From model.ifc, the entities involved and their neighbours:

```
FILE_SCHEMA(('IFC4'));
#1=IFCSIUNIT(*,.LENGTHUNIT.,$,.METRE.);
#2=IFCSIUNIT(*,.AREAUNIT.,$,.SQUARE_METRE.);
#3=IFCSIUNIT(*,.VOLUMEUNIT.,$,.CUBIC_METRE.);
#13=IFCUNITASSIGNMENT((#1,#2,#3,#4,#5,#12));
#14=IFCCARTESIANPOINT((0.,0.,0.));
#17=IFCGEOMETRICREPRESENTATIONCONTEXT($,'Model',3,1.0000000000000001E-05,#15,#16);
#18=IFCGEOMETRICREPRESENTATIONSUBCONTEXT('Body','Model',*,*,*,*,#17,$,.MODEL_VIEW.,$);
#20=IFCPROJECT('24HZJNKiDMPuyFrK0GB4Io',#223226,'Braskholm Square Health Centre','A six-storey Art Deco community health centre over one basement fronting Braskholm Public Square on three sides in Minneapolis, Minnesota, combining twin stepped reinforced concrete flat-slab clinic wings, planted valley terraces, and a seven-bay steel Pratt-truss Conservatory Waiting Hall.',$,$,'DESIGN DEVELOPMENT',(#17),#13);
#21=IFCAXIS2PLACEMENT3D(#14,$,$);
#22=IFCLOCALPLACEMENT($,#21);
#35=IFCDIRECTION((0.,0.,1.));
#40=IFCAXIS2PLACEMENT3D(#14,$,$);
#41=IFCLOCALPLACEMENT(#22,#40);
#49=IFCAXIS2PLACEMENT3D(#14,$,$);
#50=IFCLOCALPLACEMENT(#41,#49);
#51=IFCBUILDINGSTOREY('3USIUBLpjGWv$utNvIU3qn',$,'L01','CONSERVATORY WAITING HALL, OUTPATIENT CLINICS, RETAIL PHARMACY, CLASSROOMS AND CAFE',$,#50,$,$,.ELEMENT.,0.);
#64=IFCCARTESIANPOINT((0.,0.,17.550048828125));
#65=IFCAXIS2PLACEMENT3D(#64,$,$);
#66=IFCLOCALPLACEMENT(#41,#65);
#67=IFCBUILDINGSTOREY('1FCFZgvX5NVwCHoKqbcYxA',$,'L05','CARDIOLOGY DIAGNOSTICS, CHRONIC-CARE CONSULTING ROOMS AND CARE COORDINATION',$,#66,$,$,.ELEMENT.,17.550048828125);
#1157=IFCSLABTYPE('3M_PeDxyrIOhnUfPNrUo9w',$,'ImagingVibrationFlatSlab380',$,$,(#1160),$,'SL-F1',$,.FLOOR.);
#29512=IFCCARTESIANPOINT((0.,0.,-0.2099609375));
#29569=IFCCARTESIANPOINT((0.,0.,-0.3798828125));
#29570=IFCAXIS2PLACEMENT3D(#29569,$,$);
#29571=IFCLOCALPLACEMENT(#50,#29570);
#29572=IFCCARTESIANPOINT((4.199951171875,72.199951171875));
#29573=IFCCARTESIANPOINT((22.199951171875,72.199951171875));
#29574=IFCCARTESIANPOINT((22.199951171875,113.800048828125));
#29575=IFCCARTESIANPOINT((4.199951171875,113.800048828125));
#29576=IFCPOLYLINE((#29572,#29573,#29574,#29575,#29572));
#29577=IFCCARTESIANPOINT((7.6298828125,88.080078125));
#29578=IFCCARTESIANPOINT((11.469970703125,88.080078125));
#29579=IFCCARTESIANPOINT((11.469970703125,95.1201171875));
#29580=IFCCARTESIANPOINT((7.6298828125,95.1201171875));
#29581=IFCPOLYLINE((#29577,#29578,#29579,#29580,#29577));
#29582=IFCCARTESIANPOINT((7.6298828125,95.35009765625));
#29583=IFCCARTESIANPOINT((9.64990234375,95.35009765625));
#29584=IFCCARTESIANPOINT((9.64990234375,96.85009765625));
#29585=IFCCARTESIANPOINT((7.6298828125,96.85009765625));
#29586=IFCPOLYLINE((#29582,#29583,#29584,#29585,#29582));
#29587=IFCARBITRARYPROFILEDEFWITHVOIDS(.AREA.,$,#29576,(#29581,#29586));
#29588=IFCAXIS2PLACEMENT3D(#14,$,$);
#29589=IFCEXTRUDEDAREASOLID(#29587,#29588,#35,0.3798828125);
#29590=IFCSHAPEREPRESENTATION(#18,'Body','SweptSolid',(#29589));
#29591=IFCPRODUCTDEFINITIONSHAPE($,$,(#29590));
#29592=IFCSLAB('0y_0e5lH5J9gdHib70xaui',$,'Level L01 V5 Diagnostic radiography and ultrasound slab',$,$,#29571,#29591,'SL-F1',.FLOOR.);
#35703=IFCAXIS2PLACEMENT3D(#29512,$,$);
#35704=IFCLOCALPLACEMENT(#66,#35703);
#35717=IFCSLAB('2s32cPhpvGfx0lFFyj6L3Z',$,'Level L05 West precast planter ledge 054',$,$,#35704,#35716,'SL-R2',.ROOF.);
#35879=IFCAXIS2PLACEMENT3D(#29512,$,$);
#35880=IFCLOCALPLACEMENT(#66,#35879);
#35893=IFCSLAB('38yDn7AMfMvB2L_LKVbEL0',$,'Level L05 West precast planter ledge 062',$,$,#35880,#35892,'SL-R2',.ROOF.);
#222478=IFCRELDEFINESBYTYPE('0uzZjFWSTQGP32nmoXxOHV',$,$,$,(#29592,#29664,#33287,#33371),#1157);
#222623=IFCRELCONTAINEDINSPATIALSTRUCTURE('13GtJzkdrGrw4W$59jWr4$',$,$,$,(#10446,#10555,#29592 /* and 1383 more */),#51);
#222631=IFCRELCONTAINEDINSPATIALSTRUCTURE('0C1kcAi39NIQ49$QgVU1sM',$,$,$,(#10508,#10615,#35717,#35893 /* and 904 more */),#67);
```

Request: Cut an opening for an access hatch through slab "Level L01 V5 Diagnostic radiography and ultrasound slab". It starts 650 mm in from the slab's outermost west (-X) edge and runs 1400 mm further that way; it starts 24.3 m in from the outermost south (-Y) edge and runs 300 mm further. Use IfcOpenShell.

```python
import numpy as np
import ifcopenshell
import ifcopenshell.api.feature
import ifcopenshell.api.geometry
import ifcopenshell.api.root
import ifcopenshell.geom
import ifcopenshell.util.placement
import ifcopenshell.util.representation
import ifcopenshell.util.shape
import ifcopenshell.util.unit

model = ifcopenshell.open("model.ifc")
unit_scale = ifcopenshell.util.unit.calculate_unit_scale(model)
settings = ifcopenshell.geom.settings()


def volume(element):
    """Net volume in cubic metres, openings subtracted."""
    shape = ifcopenshell.geom.create_shape(settings, element)
    return ifcopenshell.util.shape.get_volume(shape.geometry)


slab = model.by_guid("0y_0e5lH5J9gdHib70xaui")
before = volume(slab)

# Extent in the slab's own axes, in metres. The edges named are its -X and -Y sides.
slab_shape = ifcopenshell.geom.create_shape(settings, slab)
vertices = ifcopenshell.util.shape.get_vertices(slab_shape.geometry)
x_min, y_min, bottom = vertices.min(axis=0)
top = vertices[:, 2].max()

opening = ifcopenshell.api.root.create_entity(model, ifc_class="IfcOpeningElement", name="Access hatch opening", predefined_type="OPENING")
context = ifcopenshell.util.representation.get_context(model, "Model", "Body", "MODEL_VIEW")
width, depth = 1.4, 0.3
outline = [(0.0, 0.0), (width, 0.0), (width, depth), (0.0, depth), (0.0, 0.0)]
# Overshoot both faces by 50 mm so the cut is clean.
shape = ifcopenshell.api.geometry.add_slab_representation(
    model, context=context, depth=top - bottom + 0.1, polyline=outline
)
ifcopenshell.api.geometry.assign_representation(model, product=opening, representation=shape)

matrix = ifcopenshell.util.placement.get_local_placement(slab.ObjectPlacement)
matrix[:, 3] = matrix @ np.append(np.array([x_min + 0.65, y_min + 24.3, bottom - 0.05]) / unit_scale, 1.0)
ifcopenshell.api.geometry.edit_object_placement(model, product=opening, matrix=matrix, is_si=False)
ifcopenshell.api.feature.add_feature(model, feature=opening, element=slab)

after = volume(slab)

print(f"slab volume {before:.3f} -> {after:.3f} m3")

model.write("model_edited.ifc")
```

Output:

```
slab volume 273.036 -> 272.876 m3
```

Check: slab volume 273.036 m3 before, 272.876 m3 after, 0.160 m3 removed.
